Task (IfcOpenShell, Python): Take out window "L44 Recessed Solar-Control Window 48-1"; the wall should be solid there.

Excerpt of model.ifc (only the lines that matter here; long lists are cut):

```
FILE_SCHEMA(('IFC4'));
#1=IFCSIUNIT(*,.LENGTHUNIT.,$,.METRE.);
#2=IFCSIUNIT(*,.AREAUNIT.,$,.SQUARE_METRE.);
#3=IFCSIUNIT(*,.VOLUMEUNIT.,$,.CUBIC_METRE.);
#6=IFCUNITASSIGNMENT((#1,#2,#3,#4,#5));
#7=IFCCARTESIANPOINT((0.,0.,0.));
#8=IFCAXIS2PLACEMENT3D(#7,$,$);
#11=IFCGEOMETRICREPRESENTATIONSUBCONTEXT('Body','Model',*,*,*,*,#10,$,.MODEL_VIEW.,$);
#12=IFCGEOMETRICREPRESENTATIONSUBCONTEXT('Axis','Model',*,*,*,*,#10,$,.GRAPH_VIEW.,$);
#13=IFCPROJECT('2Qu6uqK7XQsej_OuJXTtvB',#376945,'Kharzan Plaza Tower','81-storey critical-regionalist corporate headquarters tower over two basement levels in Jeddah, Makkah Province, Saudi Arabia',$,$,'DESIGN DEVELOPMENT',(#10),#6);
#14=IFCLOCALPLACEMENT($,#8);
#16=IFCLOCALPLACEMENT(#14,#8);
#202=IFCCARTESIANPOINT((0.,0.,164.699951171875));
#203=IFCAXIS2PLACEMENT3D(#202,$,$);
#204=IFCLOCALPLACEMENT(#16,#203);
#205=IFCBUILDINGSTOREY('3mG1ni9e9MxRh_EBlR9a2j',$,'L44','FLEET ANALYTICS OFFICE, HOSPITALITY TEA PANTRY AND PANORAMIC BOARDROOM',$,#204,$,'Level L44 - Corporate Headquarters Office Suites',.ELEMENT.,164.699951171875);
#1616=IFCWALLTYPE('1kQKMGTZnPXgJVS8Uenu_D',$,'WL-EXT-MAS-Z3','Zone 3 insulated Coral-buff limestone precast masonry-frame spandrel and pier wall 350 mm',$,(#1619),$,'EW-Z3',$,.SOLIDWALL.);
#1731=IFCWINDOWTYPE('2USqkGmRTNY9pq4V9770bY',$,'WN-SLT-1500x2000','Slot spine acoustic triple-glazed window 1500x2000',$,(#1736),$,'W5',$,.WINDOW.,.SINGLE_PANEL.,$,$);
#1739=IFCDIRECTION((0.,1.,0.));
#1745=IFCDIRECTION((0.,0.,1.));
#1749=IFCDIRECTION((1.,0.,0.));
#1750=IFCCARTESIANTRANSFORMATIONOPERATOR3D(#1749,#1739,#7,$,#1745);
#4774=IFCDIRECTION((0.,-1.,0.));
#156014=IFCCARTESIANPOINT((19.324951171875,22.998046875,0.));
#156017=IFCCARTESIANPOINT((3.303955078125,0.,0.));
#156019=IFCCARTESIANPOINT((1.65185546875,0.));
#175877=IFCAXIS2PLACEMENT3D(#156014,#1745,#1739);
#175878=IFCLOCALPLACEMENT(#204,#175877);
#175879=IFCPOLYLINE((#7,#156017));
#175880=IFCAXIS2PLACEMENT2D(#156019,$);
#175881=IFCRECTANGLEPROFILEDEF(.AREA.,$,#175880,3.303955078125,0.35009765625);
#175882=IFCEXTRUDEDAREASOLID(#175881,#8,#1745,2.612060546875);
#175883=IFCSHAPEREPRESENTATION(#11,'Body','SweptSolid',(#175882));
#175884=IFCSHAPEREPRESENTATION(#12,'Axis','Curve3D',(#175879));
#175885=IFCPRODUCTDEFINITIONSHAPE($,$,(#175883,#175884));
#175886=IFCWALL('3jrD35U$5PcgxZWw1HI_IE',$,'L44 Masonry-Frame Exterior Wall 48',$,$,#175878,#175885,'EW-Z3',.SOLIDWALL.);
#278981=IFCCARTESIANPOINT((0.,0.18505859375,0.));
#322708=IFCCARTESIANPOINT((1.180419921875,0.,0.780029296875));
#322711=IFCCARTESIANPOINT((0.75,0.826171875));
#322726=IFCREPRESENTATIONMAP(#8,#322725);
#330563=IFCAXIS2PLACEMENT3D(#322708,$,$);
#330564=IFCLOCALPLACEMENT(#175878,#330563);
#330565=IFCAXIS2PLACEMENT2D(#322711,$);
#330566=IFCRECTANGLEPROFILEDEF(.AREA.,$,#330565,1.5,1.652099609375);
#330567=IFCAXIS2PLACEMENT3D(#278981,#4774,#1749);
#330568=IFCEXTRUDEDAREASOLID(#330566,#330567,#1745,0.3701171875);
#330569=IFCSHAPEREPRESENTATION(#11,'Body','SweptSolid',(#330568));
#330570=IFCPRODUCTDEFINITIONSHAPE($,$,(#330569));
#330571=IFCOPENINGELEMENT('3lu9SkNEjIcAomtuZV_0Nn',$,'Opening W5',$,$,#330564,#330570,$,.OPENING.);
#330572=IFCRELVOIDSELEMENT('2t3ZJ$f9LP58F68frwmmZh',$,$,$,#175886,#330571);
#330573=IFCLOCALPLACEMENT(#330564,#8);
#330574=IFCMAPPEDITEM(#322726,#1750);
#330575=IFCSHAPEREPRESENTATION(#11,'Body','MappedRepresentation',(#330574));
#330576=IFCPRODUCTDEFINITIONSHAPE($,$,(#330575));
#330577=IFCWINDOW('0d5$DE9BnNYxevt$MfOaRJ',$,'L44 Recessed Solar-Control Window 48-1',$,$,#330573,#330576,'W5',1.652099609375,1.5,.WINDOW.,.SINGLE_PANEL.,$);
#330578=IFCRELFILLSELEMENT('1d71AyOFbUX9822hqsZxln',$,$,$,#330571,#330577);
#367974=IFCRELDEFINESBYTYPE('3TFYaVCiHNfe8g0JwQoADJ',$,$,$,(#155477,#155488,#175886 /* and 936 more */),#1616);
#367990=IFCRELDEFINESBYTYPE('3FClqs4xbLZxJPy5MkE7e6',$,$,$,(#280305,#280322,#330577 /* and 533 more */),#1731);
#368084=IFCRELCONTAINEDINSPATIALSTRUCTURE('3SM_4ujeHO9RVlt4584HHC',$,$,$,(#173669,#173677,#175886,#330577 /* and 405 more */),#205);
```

```python
import ifcopenshell
import ifcopenshell.api.feature
import ifcopenshell.api.root
import ifcopenshell.geom
import ifcopenshell.util.shape

model = ifcopenshell.open("model.ifc")
settings = ifcopenshell.geom.settings()


def volume(element):
    """Net volume in cubic metres, openings subtracted."""
    shape = ifcopenshell.geom.create_shape(settings, element)
    return ifcopenshell.util.shape.get_volume(shape.geometry)


window = model.by_id(330577)
opening = window.FillsVoids[0].RelatingOpeningElement
wall = opening.VoidsElements[0].RelatingBuildingElement
before = volume(wall)

ifcopenshell.api.root.remove_product(model, product=window)
ifcopenshell.api.feature.remove_feature(model, feature=opening)

after = volume(wall)

print(f"wall volume {before:.3f} -> {after:.3f} m3")

model.write("model_v2.ifc")
```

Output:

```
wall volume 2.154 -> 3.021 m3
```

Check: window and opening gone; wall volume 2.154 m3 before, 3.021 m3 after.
